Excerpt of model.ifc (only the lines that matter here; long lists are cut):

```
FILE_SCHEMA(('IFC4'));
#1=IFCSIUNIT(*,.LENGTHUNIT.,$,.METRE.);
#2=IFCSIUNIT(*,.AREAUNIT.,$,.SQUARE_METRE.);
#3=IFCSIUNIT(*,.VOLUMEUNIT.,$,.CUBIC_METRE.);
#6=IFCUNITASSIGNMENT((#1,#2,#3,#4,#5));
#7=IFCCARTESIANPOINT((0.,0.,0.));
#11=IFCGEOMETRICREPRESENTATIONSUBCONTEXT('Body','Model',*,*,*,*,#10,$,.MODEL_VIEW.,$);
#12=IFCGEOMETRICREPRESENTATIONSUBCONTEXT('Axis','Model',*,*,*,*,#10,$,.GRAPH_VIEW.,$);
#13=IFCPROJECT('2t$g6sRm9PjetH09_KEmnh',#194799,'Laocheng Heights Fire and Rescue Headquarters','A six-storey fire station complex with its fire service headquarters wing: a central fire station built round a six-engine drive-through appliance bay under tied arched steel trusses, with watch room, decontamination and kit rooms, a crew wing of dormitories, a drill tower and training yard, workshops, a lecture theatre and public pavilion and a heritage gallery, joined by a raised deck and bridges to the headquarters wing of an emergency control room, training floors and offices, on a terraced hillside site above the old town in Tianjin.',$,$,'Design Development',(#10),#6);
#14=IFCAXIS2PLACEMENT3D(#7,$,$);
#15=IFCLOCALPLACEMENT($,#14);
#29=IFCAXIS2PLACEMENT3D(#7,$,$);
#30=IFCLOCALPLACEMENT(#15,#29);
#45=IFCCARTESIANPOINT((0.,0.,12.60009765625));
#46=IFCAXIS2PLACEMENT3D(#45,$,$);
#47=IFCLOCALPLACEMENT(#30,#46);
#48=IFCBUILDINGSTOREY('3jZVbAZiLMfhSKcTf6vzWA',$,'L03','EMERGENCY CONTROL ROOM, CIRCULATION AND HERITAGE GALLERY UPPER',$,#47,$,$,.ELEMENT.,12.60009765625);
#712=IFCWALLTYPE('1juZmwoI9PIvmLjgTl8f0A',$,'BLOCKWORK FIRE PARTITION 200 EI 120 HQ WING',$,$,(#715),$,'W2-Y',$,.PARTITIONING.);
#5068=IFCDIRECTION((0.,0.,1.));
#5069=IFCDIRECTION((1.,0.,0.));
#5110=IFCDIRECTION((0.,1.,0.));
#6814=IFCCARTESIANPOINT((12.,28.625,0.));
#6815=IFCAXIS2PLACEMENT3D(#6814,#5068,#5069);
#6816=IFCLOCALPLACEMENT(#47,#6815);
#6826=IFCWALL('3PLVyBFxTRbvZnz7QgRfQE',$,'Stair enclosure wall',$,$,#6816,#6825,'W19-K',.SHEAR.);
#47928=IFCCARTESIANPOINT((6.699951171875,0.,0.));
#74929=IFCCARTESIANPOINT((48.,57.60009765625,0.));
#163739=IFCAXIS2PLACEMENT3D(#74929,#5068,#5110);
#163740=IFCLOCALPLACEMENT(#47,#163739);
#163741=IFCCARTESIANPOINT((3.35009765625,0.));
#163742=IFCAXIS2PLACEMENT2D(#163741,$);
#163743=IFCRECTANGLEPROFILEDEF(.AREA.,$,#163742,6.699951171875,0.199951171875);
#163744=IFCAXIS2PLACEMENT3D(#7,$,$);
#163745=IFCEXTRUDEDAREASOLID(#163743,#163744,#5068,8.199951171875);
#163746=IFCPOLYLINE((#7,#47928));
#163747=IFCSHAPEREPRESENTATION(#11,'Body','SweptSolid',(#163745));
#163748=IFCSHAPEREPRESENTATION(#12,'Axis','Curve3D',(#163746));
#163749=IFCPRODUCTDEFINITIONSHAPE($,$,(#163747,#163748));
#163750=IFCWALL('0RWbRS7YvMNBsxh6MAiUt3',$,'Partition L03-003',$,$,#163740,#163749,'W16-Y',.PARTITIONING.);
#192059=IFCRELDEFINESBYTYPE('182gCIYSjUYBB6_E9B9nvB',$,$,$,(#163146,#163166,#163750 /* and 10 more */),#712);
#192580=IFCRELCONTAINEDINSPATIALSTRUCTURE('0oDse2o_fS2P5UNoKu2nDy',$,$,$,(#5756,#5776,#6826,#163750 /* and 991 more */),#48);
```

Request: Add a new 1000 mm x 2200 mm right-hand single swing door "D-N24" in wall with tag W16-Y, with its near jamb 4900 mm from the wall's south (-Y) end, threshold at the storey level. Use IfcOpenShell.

```python
import numpy as np
import ifcopenshell
import ifcopenshell.api.feature
import ifcopenshell.api.geometry
import ifcopenshell.api.root
import ifcopenshell.api.spatial
import ifcopenshell.geom
import ifcopenshell.util.element
import ifcopenshell.util.placement
import ifcopenshell.util.representation
import ifcopenshell.util.shape
import ifcopenshell.util.unit

model = ifcopenshell.open("model.ifc")
unit_scale = ifcopenshell.util.unit.calculate_unit_scale(model)
settings = ifcopenshell.geom.settings()


def volume(element):
    """Net volume in cubic metres, openings subtracted."""
    shape = ifcopenshell.geom.create_shape(settings, element)
    return ifcopenshell.util.shape.get_volume(shape.geometry)


wall = model.by_id(163750)
storey = ifcopenshell.util.element.get_container(wall, ifc_class="IfcBuildingStorey")
context = ifcopenshell.util.representation.get_context(model, "Model", "Body", "MODEL_VIEW")
before = volume(wall)

width, height, from_end, sill = 1, 2.2, 4.9, 0.0  # metres

# The wall runs along its own X axis, and the end named is its -X end.
wall_shape = ifcopenshell.geom.create_shape(settings, wall)
x, y, z = ifcopenshell.util.shape.get_vertices(wall_shape.geometry).T
start = x.min() + from_end
face, thickness = float(y.min()), float(y.max() - y.min())
wall_matrix = ifcopenshell.util.placement.get_local_placement(wall.ObjectPlacement)
level = ifcopenshell.util.placement.get_local_placement(storey.ObjectPlacement)[2, 3]


def in_wall(x, y):
    """Placement at x, y metres in the wall's axes, at sill height."""
    matrix = wall_matrix.copy()
    matrix[:, 3] = wall_matrix @ np.array([x / unit_scale, y / unit_scale, 0.0, 1.0])
    matrix[2, 3] = level + sill / unit_scale
    return matrix


# Opening: a box that overshoots both wall faces by 50 mm.
opening = ifcopenshell.api.root.create_entity(model, ifc_class="IfcOpeningElement", predefined_type="OPENING")
box = ifcopenshell.api.geometry.add_wall_representation(
    model, context=context, length=width, height=height, thickness=thickness + 0.1
)
ifcopenshell.api.geometry.assign_representation(model, product=opening, representation=box)
ifcopenshell.api.geometry.edit_object_placement(model, product=opening, matrix=in_wall(start, face - 0.05), is_si=False)
ifcopenshell.api.feature.add_feature(model, feature=opening, element=wall)

door = ifcopenshell.api.root.create_entity(model, ifc_class="IfcDoor", name="D-N24", predefined_type="DOOR")
door.OverallWidth, door.OverallHeight = width / unit_scale, height / unit_scale
door.OperationType = "SINGLE_SWING_RIGHT"
body = ifcopenshell.api.geometry.add_door_representation(
    model,
    context=context,
    overall_width=door.OverallWidth,
    overall_height=door.OverallHeight,
    operation_type="SINGLE_SWING_RIGHT",
    lining_properties={"LiningDepth": thickness / unit_scale, "ThresholdDepth": thickness / unit_scale},
)
ifcopenshell.api.geometry.assign_representation(model, product=door, representation=body)
ifcopenshell.api.spatial.assign_container(model, products=[door], relating_structure=storey)
ifcopenshell.api.feature.add_filling(model, opening=opening, element=door)

# The lining spans the wall, so the door starts at the wall face.
ifcopenshell.api.geometry.edit_object_placement(model, product=door, matrix=in_wall(start, face), is_si=False)

after = volume(wall)

print(f"wall volume {before:.3f} -> {after:.3f} m3")

model.write("model_updated.ifc")
```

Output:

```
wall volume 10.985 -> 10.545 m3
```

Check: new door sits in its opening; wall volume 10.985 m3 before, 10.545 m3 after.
